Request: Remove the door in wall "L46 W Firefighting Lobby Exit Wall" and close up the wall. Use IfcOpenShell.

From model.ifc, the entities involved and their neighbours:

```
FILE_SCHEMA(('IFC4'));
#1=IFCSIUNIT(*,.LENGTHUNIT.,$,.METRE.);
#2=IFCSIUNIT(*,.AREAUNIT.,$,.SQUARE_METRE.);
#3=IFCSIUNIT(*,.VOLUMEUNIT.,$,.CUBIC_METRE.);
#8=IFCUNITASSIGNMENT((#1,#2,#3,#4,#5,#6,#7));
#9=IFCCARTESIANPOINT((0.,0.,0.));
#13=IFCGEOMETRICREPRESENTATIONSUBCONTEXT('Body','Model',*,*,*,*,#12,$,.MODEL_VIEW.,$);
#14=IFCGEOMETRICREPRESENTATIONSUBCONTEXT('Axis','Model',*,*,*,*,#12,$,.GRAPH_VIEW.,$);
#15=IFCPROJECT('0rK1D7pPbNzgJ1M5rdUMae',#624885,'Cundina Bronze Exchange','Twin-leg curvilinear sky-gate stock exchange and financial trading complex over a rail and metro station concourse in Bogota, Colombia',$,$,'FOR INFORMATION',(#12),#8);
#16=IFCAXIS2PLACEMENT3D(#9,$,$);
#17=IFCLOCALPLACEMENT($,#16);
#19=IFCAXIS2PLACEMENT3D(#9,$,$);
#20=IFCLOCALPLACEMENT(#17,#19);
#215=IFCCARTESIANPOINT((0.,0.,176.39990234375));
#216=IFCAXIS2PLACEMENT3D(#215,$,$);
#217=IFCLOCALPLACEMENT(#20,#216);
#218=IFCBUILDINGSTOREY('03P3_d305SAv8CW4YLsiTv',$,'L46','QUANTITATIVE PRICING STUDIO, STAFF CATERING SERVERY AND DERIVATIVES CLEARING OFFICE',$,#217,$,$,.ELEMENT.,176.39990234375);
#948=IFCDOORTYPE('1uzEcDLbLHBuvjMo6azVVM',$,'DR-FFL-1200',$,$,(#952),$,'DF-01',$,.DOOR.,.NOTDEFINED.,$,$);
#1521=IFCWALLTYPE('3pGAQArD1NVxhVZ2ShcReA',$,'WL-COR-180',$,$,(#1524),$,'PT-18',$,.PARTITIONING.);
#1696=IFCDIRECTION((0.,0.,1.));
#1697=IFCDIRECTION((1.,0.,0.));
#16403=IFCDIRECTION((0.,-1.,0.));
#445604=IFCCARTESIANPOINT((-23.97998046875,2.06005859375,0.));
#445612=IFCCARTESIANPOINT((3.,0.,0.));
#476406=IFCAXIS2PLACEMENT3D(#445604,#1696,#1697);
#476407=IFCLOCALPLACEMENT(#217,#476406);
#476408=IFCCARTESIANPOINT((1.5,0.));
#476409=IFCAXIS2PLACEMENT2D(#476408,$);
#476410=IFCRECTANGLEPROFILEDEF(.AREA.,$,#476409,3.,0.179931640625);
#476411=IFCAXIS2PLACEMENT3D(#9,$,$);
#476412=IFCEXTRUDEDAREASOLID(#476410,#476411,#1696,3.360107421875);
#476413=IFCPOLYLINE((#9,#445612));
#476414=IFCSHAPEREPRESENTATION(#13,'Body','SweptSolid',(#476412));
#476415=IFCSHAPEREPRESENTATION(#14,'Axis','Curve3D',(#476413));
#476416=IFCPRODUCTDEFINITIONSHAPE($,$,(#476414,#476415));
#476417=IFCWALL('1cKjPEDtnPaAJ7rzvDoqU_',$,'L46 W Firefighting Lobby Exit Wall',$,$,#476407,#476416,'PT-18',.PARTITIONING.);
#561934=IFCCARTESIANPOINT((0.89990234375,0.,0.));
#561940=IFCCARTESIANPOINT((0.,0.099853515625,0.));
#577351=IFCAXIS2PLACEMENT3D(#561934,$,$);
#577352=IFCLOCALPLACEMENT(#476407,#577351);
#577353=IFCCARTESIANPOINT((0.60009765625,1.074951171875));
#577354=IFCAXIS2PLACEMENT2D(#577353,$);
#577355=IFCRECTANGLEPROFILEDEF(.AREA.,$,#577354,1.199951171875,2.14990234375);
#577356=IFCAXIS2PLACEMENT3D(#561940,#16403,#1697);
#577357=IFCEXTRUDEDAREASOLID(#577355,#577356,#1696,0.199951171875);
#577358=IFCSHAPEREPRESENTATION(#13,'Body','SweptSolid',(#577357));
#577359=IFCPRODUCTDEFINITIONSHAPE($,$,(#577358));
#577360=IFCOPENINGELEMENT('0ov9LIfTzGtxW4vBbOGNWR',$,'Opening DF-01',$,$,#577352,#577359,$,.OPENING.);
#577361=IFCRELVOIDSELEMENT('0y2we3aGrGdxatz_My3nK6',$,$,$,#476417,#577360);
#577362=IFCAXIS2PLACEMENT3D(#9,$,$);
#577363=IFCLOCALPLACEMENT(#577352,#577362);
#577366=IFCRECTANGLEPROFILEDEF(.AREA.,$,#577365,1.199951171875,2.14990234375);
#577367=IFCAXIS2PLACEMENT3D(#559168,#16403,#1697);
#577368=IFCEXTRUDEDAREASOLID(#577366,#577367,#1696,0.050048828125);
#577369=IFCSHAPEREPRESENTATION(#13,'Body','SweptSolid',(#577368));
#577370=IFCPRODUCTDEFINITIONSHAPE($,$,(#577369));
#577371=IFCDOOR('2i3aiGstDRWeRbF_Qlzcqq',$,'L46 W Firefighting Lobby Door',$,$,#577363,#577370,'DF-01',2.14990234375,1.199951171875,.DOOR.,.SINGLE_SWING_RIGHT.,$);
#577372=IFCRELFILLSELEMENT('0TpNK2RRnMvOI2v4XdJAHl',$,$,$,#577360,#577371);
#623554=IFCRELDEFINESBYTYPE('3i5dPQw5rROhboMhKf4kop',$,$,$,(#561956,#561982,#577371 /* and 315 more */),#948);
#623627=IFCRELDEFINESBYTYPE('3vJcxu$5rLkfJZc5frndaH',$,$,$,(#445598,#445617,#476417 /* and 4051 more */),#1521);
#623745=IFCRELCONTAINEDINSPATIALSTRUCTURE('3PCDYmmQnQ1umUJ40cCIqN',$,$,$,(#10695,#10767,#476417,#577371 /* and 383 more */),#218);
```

```python
import ifcopenshell
import ifcopenshell.api.feature
import ifcopenshell.api.root
import ifcopenshell.geom
import ifcopenshell.util.shape

model = ifcopenshell.open("model.ifc")
settings = ifcopenshell.geom.settings()


def volume(element):
    """Net volume in cubic metres, openings subtracted."""
    shape = ifcopenshell.geom.create_shape(settings, element)
    return ifcopenshell.util.shape.get_volume(shape.geometry)


door = model.by_guid("2i3aiGstDRWeRbF_Qlzcqq")
opening = door.FillsVoids[0].RelatingOpeningElement
wall = opening.VoidsElements[0].RelatingBuildingElement
before = volume(wall)

ifcopenshell.api.root.remove_product(model, product=door)
ifcopenshell.api.feature.remove_feature(model, feature=opening)

after = volume(wall)

print(f"wall volume {before:.3f} -> {after:.3f} m3")

model.write("model_updated.ifc")
```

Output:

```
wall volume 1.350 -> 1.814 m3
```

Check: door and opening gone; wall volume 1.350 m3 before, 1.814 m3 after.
